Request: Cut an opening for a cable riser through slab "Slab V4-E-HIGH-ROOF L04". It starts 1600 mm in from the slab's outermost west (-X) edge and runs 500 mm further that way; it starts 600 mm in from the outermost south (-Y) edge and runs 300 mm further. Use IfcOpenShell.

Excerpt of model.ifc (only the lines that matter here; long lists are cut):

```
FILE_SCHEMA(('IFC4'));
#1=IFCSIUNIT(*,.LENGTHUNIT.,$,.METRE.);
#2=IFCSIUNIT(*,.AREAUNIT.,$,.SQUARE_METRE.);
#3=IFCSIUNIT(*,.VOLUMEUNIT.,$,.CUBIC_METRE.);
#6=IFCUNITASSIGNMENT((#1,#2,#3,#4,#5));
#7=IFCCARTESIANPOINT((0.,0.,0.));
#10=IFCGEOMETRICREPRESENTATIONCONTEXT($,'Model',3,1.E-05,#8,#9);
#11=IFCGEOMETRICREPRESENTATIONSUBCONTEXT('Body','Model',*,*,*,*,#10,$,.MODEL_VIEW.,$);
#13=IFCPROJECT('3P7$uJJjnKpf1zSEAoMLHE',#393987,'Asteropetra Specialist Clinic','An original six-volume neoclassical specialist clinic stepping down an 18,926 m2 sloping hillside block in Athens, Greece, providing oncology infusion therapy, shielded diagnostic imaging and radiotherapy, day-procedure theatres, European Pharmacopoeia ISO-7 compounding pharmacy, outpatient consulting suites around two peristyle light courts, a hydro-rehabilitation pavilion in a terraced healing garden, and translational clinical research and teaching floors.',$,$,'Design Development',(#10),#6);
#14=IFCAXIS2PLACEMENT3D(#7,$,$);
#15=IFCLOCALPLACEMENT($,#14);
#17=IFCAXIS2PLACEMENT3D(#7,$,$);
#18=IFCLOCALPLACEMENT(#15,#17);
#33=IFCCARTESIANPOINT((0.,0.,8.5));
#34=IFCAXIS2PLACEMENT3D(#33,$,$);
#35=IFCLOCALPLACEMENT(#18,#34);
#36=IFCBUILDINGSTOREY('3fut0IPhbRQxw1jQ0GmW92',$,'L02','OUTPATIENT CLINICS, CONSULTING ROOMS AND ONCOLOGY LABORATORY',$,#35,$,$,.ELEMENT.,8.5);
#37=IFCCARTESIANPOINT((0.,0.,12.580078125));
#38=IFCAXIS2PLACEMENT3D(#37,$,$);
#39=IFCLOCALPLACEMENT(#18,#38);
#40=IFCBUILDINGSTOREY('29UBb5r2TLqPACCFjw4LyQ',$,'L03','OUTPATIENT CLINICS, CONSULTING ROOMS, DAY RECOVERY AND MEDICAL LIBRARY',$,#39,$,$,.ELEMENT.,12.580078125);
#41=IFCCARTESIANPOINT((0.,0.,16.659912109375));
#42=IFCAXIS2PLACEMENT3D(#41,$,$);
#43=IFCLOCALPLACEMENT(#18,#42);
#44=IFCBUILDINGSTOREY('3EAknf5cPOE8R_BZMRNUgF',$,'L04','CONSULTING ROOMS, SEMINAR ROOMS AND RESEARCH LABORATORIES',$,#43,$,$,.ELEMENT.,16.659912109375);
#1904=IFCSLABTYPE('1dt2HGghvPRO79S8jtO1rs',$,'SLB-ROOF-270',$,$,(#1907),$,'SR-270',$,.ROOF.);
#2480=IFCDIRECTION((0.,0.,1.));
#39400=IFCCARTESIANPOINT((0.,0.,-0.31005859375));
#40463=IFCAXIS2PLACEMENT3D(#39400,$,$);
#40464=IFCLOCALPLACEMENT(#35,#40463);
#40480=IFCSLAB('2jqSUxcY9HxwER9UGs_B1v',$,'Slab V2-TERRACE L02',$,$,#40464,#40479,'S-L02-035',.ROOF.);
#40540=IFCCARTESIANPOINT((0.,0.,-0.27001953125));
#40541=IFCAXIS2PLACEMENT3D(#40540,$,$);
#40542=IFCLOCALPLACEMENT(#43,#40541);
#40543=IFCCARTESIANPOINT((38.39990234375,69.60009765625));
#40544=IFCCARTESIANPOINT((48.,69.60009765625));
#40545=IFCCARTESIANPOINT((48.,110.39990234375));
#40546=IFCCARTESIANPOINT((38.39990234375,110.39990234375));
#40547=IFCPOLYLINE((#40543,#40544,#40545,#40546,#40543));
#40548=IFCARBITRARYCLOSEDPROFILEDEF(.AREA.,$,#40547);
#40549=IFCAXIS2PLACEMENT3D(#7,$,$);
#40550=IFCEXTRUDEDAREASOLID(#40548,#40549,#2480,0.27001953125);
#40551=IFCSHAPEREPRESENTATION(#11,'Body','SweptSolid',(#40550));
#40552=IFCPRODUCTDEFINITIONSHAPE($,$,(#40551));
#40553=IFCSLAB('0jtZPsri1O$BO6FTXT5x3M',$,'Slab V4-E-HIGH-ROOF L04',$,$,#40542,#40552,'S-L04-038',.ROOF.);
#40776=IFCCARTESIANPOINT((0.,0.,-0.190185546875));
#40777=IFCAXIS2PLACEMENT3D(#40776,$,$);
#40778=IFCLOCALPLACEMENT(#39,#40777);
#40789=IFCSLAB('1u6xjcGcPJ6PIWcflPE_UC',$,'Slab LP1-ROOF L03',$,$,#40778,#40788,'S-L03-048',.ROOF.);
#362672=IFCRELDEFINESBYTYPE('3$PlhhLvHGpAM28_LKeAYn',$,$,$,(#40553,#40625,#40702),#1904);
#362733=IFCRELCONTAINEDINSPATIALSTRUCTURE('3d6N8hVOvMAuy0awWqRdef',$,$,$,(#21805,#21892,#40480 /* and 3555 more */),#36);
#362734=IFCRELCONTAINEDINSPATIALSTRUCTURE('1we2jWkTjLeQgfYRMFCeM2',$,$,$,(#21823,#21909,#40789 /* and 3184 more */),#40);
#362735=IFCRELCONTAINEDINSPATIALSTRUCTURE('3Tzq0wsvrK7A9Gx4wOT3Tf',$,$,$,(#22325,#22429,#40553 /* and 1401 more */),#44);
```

```python
import numpy as np
import ifcopenshell
import ifcopenshell.api.feature
import ifcopenshell.api.geometry
import ifcopenshell.api.root
import ifcopenshell.geom
import ifcopenshell.util.placement
import ifcopenshell.util.representation
import ifcopenshell.util.shape
import ifcopenshell.util.unit

model = ifcopenshell.open("model.ifc")
unit_scale = ifcopenshell.util.unit.calculate_unit_scale(model)
settings = ifcopenshell.geom.settings()


def volume(element):
    """Net volume in cubic metres, openings subtracted."""
    shape = ifcopenshell.geom.create_shape(settings, element)
    return ifcopenshell.util.shape.get_volume(shape.geometry)


slab = model.by_guid("0jtZPsri1O$BO6FTXT5x3M")
before = volume(slab)

# Extent in the slab's own axes, in metres. The edges named are its -X and -Y sides.
slab_shape = ifcopenshell.geom.create_shape(settings, slab)
vertices = ifcopenshell.util.shape.get_vertices(slab_shape.geometry)
x_min, y_min, bottom = vertices.min(axis=0)
top = vertices[:, 2].max()

opening = ifcopenshell.api.root.create_entity(model, ifc_class="IfcOpeningElement", name="Cable riser opening", predefined_type="OPENING")
context = ifcopenshell.util.representation.get_context(model, "Model", "Body", "MODEL_VIEW")
width, depth = 0.5, 0.3
outline = [(0.0, 0.0), (width, 0.0), (width, depth), (0.0, depth), (0.0, 0.0)]
# Overshoot both faces by 50 mm so the cut is clean.
shape = ifcopenshell.api.geometry.add_slab_representation(
    model, context=context, depth=top - bottom + 0.1, polyline=outline
)
ifcopenshell.api.geometry.assign_representation(model, product=opening, representation=shape)

matrix = ifcopenshell.util.placement.get_local_placement(slab.ObjectPlacement)
matrix[:, 3] = matrix @ np.append(np.array([x_min + 1.6, y_min + 0.6, bottom - 0.05]) / unit_scale, 1.0)
ifcopenshell.api.geometry.edit_object_placement(model, product=opening, matrix=matrix, is_si=False)
ifcopenshell.api.feature.add_feature(model, feature=opening, element=slab)

after = volume(slab)

print(f"slab volume {before:.3f} -> {after:.3f} m3")

model.write("model-out.ifc")
```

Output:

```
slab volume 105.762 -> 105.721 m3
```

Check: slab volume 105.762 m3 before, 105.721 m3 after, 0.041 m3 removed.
